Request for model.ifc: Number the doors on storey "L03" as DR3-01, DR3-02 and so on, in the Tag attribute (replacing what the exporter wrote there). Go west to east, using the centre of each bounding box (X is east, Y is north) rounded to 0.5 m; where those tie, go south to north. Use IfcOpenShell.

First a look at what the model holds.

```python
import ifcopenshell
import ifcopenshell.util.element
import ifcopenshell.util.placement

model = ifcopenshell.open("model.ifc")
print(model.schema)
storey = next(s for s in model.by_type("IfcBuildingStorey") if s.Name == "L03")
doors = [e for e in ifcopenshell.util.element.get_decomposition(storey) if e.is_a("IfcDoor")]
for e in sorted(doors, key=lambda e: e.id()):
    origin = ifcopenshell.util.placement.get_local_placement(e.ObjectPlacement)[:3, 3]
    print(e.id(), e.Tag, e.Name, origin.round(2) + 0.0, sep=" | ")
```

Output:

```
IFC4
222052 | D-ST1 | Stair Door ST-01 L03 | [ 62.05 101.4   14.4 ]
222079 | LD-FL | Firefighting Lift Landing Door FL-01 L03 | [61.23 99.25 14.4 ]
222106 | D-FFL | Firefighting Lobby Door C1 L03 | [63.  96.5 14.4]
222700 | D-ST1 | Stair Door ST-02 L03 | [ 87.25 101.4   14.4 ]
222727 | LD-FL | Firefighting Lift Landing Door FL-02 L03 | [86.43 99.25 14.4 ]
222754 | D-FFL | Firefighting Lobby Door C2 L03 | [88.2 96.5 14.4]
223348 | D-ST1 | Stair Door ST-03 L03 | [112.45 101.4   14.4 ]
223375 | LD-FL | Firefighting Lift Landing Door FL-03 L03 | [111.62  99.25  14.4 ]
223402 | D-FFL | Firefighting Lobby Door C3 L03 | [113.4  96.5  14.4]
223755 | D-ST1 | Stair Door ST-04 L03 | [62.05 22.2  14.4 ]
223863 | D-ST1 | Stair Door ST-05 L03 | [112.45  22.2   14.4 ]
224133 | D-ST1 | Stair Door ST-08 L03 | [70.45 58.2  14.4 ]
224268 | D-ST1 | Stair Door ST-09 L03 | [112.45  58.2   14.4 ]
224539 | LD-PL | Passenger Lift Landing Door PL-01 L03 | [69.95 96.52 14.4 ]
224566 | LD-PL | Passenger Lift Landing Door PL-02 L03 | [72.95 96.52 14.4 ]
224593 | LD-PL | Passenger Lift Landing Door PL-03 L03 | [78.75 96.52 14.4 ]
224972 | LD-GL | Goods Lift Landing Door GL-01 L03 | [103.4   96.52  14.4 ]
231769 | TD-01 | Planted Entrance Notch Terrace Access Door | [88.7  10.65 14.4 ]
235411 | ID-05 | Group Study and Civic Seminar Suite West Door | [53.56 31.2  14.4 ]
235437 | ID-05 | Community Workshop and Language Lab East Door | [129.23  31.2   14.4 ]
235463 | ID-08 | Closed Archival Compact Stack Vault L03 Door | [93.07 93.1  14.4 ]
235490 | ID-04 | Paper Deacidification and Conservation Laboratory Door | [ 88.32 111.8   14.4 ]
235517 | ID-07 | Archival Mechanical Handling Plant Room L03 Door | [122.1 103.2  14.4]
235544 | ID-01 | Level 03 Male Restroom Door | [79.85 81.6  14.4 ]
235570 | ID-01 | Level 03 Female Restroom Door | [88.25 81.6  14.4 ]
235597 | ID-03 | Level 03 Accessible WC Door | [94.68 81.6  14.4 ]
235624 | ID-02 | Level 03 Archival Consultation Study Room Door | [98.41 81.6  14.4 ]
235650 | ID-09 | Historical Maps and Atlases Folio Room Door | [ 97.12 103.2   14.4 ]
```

```python
import ifcopenshell
import ifcopenshell.geom
import ifcopenshell.util.element
import ifcopenshell.util.shape

model = ifcopenshell.open("model.ifc")
settings = ifcopenshell.geom.settings()
settings.set("use-world-coords", True)


def centre(element):
    shape = ifcopenshell.geom.create_shape(settings, element)
    return ifcopenshell.util.shape.get_bbox_centroid(shape.geometry)


storey = next(s for s in model.by_type("IfcBuildingStorey") if s.Name == "L03")
doors = [e for e in ifcopenshell.util.element.get_decomposition(storey) if e.is_a("IfcDoor")]

# Insertion points can sit at a corner or the storey origin, so sort by the geometry (in metres).
centres = {e: centre(e) for e in doors}
doors.sort(key=lambda e: (round(centres[e][0] / 0.5), centres[e][1]))

for i, e in enumerate(doors, start=1):
    number = f"DR3-{i:02d}"
    e.Tag = number
    print(e.id(), number)

model.write("model_updated.ifc")
```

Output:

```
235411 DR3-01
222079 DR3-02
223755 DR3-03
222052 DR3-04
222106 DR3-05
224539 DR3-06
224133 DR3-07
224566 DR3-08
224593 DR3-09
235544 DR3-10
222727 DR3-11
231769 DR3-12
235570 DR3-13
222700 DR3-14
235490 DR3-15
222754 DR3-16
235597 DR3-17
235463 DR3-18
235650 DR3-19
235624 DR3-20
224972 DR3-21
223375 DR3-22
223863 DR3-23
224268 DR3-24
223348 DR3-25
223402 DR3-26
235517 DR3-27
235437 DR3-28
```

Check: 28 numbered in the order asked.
